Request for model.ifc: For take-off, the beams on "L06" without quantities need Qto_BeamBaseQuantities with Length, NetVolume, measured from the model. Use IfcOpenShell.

First a look at what the model holds.

```python
import ifcopenshell
import ifcopenshell.util.element
import ifcopenshell.util.unit

model = ifcopenshell.open("model.ifc")
print(model.schema)
for unit_type in ("LENGTHUNIT", "AREAUNIT", "VOLUMEUNIT"):
    print(unit_type, ifcopenshell.util.unit.calculate_unit_scale(model, unit_type))
storey = next(s for s in model.by_type("IfcBuildingStorey") if s.Name == "L06")
beams = [e for e in ifcopenshell.util.element.get_decomposition(storey) if e.is_a("IfcBeam")]
for e in sorted(beams, key=lambda e: e.id()):
    print(e.id(), e.is_a(), e.Name, list(ifcopenshell.util.element.get_psets(e, qtos_only=True)), sep=" | ")
```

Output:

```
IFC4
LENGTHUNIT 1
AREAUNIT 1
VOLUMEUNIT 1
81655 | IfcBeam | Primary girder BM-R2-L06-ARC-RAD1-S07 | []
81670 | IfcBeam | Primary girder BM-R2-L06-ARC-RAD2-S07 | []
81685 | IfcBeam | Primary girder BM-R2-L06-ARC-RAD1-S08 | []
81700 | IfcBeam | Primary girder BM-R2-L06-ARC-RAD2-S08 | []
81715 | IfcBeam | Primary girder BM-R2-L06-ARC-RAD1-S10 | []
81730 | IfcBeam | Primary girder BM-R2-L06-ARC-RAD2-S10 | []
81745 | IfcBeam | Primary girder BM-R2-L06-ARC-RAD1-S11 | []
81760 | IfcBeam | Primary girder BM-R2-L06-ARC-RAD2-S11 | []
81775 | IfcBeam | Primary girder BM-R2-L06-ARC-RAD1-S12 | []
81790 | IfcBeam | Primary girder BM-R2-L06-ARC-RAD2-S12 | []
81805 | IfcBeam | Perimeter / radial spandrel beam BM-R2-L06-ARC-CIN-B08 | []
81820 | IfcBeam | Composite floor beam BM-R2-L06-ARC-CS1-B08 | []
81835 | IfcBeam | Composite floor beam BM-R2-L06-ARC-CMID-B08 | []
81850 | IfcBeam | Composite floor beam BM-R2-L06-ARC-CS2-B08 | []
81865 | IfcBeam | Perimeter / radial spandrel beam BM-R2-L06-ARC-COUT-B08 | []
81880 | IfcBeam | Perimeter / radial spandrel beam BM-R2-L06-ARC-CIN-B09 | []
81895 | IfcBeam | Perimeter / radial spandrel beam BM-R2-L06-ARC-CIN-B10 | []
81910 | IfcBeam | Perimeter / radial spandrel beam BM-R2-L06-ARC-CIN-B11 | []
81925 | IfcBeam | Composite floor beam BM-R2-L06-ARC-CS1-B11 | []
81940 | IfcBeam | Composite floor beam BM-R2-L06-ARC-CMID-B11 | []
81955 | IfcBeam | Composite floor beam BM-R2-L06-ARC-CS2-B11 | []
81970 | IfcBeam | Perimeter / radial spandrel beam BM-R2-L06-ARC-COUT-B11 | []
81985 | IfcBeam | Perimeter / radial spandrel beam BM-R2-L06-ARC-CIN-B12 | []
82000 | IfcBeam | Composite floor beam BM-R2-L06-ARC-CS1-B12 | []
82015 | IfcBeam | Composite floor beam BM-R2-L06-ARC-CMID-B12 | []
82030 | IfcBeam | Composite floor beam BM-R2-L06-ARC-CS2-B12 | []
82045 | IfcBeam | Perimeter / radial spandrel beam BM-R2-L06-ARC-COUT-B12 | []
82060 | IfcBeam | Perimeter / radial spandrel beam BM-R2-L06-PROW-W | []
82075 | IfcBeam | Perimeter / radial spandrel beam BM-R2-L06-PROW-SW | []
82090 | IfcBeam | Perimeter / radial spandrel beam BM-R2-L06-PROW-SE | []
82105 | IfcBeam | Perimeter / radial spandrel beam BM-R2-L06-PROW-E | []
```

```python
import ifcopenshell
import ifcopenshell.api.pset
import ifcopenshell.geom
import ifcopenshell.util.element
import ifcopenshell.util.shape
import ifcopenshell.util.unit

model = ifcopenshell.open("model.ifc")
unit_scale = ifcopenshell.util.unit.calculate_unit_scale(model)
volume_scale = ifcopenshell.util.unit.calculate_unit_scale(model, "VOLUMEUNIT")
settings = ifcopenshell.geom.settings()

storey = next(s for s in model.by_type("IfcBuildingStorey") if s.Name == "L06")
beams = [e for e in ifcopenshell.util.element.get_decomposition(storey) if e.is_a("IfcBeam")]

for e in sorted(beams, key=lambda e: e.id()):
    if ifcopenshell.util.element.get_psets(e, qtos_only=True, should_inherit=False):
        continue
    # Geometry comes back in metres, in the element's own axes.
    shape = ifcopenshell.geom.create_shape(settings, e)
    values = {
        "Length": ifcopenshell.util.shape.get_max_xyz(shape.geometry) / unit_scale,
        "NetVolume": ifcopenshell.util.shape.get_volume(shape.geometry) / volume_scale,
    }
    qto = ifcopenshell.api.pset.add_qto(model, product=e, name="Qto_BeamBaseQuantities")
    ifcopenshell.api.pset.edit_qto(model, qto=qto, properties=values)
    print(e.id(), {k: round(v, 3) for k, v in values.items()})

model.write("model_updated.ifc")
```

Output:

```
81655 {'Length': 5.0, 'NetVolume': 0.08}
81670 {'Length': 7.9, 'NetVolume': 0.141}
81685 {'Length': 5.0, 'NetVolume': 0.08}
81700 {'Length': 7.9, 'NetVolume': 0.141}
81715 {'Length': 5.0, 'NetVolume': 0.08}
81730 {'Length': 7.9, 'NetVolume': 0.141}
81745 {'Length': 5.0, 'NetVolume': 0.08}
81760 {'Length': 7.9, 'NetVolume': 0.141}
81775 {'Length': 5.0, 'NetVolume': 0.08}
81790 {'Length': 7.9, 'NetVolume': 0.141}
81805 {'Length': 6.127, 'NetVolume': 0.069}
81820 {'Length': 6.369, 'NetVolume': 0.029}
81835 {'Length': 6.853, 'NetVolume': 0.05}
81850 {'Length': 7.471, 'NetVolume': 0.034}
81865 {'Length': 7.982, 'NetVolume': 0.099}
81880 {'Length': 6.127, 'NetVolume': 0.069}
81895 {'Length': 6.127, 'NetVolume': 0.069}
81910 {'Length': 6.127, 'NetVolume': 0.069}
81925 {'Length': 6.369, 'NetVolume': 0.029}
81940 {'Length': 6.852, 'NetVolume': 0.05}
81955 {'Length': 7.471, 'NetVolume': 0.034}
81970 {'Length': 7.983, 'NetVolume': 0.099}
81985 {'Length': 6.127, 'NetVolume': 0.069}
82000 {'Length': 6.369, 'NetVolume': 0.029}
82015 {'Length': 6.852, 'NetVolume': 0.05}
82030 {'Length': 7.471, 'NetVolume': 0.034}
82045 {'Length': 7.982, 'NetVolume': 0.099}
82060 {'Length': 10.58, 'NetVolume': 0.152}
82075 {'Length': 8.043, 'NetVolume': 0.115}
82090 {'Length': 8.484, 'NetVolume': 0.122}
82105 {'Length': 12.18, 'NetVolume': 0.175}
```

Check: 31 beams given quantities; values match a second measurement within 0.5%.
